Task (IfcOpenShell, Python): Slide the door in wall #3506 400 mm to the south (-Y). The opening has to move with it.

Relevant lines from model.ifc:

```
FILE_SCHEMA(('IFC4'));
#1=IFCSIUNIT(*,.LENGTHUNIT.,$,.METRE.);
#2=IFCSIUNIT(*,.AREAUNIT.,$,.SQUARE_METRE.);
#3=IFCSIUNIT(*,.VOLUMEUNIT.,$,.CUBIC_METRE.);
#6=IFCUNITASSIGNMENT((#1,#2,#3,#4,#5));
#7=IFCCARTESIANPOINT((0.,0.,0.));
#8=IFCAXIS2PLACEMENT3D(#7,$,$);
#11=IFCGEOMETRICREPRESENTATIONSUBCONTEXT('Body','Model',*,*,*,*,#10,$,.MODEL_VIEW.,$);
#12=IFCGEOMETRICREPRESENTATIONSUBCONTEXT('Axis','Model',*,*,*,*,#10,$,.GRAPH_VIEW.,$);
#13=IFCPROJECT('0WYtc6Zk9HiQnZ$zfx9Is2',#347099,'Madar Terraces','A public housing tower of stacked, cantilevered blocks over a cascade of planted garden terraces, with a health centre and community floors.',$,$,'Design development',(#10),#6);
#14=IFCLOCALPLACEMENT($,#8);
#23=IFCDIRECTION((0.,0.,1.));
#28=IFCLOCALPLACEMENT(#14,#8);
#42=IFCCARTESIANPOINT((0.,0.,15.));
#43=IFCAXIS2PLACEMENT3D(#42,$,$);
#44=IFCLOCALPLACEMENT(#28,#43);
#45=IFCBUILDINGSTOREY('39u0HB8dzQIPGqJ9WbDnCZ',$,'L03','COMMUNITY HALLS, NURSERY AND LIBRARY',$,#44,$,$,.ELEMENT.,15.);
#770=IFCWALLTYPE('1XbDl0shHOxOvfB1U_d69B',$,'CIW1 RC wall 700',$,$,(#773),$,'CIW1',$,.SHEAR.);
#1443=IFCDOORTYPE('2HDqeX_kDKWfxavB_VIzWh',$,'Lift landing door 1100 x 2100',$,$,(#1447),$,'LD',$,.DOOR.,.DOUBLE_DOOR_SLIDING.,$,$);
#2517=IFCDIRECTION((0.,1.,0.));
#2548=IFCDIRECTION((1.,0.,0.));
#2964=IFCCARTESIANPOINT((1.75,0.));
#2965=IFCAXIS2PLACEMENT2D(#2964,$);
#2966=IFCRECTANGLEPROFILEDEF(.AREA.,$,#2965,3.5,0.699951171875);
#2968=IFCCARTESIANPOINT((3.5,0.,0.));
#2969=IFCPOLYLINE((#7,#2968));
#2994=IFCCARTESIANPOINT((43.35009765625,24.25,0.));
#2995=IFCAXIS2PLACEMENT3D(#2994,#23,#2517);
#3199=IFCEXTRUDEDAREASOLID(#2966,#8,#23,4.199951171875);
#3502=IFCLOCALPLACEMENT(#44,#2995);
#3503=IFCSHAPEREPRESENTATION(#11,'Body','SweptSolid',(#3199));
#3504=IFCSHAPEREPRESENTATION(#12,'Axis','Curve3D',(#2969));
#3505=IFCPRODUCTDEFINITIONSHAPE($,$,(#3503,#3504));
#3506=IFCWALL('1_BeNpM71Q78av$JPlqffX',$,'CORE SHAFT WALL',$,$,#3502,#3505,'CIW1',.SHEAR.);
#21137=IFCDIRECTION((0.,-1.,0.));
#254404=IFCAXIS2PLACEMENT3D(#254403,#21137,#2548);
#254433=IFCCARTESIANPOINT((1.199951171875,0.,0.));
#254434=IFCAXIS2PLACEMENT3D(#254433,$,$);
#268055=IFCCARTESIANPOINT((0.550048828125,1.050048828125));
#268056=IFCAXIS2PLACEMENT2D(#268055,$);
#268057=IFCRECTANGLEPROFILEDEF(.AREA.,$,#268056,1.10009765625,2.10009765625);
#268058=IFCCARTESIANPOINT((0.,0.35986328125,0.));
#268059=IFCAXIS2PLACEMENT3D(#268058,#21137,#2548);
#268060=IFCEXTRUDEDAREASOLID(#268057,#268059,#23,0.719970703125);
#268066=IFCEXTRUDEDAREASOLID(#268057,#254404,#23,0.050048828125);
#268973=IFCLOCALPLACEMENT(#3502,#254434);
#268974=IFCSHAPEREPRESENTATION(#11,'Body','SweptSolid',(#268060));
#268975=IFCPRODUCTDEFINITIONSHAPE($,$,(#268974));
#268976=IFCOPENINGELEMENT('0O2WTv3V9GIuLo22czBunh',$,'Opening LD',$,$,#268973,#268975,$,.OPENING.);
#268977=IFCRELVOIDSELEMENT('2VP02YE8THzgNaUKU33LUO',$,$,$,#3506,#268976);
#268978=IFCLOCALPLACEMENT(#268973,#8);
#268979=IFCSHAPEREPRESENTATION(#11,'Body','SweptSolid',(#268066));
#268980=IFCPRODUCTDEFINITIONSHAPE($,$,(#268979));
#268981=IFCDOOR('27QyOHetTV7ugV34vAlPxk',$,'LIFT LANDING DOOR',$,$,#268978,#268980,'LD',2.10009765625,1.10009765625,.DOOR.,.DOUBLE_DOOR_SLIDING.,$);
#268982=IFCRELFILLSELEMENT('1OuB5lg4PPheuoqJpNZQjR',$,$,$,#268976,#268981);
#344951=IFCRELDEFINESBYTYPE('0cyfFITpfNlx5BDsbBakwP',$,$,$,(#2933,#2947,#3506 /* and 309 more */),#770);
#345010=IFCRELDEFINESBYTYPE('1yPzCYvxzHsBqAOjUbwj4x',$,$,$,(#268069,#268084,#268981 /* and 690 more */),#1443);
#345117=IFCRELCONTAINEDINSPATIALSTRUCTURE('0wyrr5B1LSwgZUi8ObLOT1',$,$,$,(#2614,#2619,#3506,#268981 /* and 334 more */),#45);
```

```python
import ifcopenshell
import ifcopenshell.api.geometry
import ifcopenshell.util.placement

model = ifcopenshell.open("model.ifc")

door = model.by_guid("27QyOHetTV7ugV34vAlPxk")
opening = door.FillsVoids[0].RelatingOpeningElement
wall = opening.VoidsElements[0].RelatingBuildingElement

wall_matrix = ifcopenshell.util.placement.get_local_placement(wall.ObjectPlacement)
shift = wall_matrix[:3, 0] * -0.4
before = ifcopenshell.util.placement.get_local_placement(door.ObjectPlacement)[:3, 3].copy()

# The door is placed relative to its opening, so it follows when the opening moves.
matrix = ifcopenshell.util.placement.get_local_placement(opening.ObjectPlacement)
matrix[:3, 3] += shift
ifcopenshell.api.geometry.edit_object_placement(
    model, product=opening, matrix=matrix, is_si=False, should_transform_children=True
)

after = ifcopenshell.util.placement.get_local_placement(door.ObjectPlacement)[:3, 3]
print("door moved by", (after - before).round(3) + 0.0)

model.write("model_edited.ifc")
```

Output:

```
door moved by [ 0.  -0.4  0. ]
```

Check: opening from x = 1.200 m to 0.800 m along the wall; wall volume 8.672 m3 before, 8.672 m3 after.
